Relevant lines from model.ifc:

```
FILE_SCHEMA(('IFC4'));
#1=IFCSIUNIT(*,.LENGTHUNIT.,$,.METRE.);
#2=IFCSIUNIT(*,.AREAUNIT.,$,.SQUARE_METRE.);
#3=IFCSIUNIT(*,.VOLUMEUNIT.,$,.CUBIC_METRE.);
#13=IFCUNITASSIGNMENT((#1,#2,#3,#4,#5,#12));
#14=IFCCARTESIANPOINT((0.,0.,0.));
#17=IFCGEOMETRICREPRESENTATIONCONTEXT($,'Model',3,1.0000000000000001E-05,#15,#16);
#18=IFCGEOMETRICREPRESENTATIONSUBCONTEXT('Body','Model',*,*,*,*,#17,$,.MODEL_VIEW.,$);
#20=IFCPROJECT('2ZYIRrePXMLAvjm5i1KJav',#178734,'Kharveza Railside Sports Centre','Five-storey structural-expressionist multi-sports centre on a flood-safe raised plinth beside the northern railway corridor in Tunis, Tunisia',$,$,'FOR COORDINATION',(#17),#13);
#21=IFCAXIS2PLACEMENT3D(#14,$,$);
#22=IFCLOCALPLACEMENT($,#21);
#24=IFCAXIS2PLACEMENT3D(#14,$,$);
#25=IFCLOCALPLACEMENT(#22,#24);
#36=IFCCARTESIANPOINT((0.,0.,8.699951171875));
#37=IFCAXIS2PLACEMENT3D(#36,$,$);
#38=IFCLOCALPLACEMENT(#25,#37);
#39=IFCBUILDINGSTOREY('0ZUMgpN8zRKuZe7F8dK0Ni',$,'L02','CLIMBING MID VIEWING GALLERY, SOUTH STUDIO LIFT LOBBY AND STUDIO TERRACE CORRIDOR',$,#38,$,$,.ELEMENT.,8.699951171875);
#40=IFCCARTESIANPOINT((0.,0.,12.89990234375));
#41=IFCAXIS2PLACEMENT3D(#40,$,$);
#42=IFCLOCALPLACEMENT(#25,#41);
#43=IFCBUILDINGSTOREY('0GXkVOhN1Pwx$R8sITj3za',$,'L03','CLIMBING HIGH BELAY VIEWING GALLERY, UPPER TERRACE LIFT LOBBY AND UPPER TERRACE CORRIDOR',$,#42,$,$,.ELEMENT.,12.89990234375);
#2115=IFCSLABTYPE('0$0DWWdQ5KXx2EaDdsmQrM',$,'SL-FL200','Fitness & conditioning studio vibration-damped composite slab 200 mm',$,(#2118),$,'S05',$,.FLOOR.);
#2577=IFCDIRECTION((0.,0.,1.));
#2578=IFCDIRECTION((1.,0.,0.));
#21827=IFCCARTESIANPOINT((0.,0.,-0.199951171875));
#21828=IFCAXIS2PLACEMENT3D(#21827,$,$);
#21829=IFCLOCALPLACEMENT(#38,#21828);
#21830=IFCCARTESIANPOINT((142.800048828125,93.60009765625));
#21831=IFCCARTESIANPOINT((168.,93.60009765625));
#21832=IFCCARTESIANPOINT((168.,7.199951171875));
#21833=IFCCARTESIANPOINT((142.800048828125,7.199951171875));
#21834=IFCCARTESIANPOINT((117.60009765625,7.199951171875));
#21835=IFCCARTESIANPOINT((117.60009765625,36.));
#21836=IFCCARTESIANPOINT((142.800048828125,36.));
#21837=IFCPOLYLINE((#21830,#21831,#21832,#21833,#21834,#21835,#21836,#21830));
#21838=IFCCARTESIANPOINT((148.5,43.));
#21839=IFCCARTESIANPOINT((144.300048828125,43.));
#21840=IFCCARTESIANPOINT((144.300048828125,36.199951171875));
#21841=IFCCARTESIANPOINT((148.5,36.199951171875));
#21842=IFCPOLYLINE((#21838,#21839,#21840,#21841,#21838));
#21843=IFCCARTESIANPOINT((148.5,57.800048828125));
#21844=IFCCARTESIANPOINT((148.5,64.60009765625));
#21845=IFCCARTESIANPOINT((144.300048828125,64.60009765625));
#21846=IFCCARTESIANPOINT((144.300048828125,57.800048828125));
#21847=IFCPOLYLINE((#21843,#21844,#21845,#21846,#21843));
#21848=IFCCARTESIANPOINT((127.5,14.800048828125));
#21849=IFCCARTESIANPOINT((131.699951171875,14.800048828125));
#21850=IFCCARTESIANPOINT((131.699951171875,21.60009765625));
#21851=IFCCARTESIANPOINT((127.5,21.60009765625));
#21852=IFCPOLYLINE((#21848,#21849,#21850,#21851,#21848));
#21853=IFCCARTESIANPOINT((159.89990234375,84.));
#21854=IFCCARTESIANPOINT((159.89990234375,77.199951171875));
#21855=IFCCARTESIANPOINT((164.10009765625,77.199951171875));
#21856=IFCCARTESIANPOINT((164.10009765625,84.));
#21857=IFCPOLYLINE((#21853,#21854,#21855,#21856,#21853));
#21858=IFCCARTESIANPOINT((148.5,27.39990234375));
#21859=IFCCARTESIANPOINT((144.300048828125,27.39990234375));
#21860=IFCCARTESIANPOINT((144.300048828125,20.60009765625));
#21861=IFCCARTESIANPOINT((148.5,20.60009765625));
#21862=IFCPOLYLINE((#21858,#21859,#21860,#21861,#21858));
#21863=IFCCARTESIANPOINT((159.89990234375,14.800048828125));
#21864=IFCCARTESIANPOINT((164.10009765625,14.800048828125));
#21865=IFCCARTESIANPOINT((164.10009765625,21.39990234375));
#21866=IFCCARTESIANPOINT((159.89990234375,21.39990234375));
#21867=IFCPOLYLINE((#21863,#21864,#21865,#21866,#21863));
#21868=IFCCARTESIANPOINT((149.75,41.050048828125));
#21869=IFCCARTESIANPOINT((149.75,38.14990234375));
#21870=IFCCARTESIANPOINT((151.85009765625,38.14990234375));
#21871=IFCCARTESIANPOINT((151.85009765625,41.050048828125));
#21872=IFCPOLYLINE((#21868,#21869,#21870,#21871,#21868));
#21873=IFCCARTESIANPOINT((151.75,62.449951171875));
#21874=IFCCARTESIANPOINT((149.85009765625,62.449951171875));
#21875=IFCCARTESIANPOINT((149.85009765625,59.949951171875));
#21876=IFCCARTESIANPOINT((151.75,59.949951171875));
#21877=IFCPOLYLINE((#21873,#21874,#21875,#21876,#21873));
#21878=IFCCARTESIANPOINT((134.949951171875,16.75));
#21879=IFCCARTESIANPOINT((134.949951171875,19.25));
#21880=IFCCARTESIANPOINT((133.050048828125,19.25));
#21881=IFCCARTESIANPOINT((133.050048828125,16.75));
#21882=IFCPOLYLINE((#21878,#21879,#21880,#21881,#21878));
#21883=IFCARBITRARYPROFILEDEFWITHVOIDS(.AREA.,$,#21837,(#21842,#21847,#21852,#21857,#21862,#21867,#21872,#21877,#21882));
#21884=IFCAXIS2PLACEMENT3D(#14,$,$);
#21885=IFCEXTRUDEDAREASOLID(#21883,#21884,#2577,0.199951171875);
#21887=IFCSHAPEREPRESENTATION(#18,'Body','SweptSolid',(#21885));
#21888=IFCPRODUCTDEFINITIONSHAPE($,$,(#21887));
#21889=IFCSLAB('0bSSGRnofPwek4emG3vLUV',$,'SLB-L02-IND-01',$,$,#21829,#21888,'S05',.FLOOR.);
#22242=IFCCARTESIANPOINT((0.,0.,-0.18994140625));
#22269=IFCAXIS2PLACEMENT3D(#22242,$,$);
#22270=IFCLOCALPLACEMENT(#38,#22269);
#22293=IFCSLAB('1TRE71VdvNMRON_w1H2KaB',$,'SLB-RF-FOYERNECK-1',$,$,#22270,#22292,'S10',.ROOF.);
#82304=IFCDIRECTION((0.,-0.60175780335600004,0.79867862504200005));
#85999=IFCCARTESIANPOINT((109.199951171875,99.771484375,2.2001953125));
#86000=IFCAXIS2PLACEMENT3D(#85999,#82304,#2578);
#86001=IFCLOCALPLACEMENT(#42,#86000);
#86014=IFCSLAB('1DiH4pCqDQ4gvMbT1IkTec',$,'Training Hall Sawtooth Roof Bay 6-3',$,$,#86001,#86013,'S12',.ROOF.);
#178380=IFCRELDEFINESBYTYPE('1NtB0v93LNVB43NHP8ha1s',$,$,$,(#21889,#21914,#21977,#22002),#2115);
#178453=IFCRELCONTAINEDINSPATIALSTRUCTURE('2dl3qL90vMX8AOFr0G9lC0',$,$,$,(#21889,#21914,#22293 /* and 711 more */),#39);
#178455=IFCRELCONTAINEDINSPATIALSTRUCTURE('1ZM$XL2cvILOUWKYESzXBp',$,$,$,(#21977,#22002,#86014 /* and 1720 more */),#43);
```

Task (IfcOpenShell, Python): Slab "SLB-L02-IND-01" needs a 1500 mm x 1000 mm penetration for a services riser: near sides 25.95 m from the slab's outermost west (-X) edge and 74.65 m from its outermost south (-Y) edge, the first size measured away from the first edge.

```python
import numpy as np
import ifcopenshell
import ifcopenshell.api.feature
import ifcopenshell.api.geometry
import ifcopenshell.api.root
import ifcopenshell.geom
import ifcopenshell.util.placement
import ifcopenshell.util.representation
import ifcopenshell.util.shape
import ifcopenshell.util.unit

model = ifcopenshell.open("model.ifc")
unit_scale = ifcopenshell.util.unit.calculate_unit_scale(model)
settings = ifcopenshell.geom.settings()


def volume(element):
    """Net volume in cubic metres, openings subtracted."""
    shape = ifcopenshell.geom.create_shape(settings, element)
    return ifcopenshell.util.shape.get_volume(shape.geometry)


slab = model.by_guid("0bSSGRnofPwek4emG3vLUV")
before = volume(slab)

# Extent in the slab's own axes, in metres. The edges named are its -X and -Y sides.
slab_shape = ifcopenshell.geom.create_shape(settings, slab)
vertices = ifcopenshell.util.shape.get_vertices(slab_shape.geometry)
x_min, y_min, bottom = vertices.min(axis=0)
top = vertices[:, 2].max()

opening = ifcopenshell.api.root.create_entity(model, ifc_class="IfcOpeningElement", name="Services riser opening", predefined_type="OPENING")
context = ifcopenshell.util.representation.get_context(model, "Model", "Body", "MODEL_VIEW")
width, depth = 1.5, 1
outline = [(0.0, 0.0), (width, 0.0), (width, depth), (0.0, depth), (0.0, 0.0)]
# Overshoot both faces by 50 mm so the cut is clean.
shape = ifcopenshell.api.geometry.add_slab_representation(
    model, context=context, depth=top - bottom + 0.1, polyline=outline
)
ifcopenshell.api.geometry.assign_representation(model, product=opening, representation=shape)

matrix = ifcopenshell.util.placement.get_local_placement(slab.ObjectPlacement)
matrix[:, 3] = matrix @ np.append(np.array([x_min + 25.95, y_min + 74.65, bottom - 0.05]) / unit_scale, 1.0)
ifcopenshell.api.geometry.edit_object_placement(model, product=opening, matrix=matrix, is_si=False)
ifcopenshell.api.feature.add_feature(model, feature=opening, element=slab)

after = volume(slab)

print(f"slab volume {before:.3f} -> {after:.3f} m3")

model.write("model_v2.ifc")
```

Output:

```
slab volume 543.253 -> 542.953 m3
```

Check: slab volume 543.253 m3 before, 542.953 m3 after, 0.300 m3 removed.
